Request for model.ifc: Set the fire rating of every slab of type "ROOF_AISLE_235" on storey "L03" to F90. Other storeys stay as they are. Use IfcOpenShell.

First a look at what the model holds.

```python
import ifcopenshell
import ifcopenshell.util.element

model = ifcopenshell.open("model.ifc")
print(model.schema)
storey = next(s for s in model.by_type("IfcBuildingStorey") if s.Name == "L03")
slabs = [e for e in ifcopenshell.util.element.get_decomposition(storey) if e.is_a("IfcSlab")]
seen = {}
for e in slabs:
    element_type = ifcopenshell.util.element.get_type(e)
    key = (element_type.Name if element_type != e and element_type else None, ifcopenshell.util.element.get_pset(e, "Pset_SlabCommon", "FireRating"))
    seen[key] = seen.get(key, 0) + 1
for (name, value), count in sorted(seen.items(), key=str):
    print(count, "x", name, "|", value)
```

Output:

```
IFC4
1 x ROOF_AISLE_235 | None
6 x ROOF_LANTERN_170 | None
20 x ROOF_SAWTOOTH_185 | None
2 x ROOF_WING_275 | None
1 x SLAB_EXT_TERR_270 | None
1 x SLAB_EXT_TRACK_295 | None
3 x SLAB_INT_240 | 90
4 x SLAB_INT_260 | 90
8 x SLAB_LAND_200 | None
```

```python
import ifcopenshell
import ifcopenshell.api.pset
import ifcopenshell.util.element

model = ifcopenshell.open("model.ifc")

storey = next(s for s in model.by_type("IfcBuildingStorey") if s.Name == "L03")
slabs = [e for e in ifcopenshell.util.element.get_decomposition(storey) if e.is_a("IfcSlab")]

count = 0
for e in slabs:
    element_type = ifcopenshell.util.element.get_type(e)
    if element_type in (None, e) or element_type.Name != "ROOF_AISLE_235":
        continue
    # add_pset returns the element's existing set when there is one.
    pset = ifcopenshell.api.pset.add_pset(model, product=e, name="Pset_SlabCommon")
    ifcopenshell.api.pset.edit_pset(model, pset=pset, properties={"FireRating": "F90"})
    count += 1

print(count, "slabs updated")

model.write("model-out.ifc")
```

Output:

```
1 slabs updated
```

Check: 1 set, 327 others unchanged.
